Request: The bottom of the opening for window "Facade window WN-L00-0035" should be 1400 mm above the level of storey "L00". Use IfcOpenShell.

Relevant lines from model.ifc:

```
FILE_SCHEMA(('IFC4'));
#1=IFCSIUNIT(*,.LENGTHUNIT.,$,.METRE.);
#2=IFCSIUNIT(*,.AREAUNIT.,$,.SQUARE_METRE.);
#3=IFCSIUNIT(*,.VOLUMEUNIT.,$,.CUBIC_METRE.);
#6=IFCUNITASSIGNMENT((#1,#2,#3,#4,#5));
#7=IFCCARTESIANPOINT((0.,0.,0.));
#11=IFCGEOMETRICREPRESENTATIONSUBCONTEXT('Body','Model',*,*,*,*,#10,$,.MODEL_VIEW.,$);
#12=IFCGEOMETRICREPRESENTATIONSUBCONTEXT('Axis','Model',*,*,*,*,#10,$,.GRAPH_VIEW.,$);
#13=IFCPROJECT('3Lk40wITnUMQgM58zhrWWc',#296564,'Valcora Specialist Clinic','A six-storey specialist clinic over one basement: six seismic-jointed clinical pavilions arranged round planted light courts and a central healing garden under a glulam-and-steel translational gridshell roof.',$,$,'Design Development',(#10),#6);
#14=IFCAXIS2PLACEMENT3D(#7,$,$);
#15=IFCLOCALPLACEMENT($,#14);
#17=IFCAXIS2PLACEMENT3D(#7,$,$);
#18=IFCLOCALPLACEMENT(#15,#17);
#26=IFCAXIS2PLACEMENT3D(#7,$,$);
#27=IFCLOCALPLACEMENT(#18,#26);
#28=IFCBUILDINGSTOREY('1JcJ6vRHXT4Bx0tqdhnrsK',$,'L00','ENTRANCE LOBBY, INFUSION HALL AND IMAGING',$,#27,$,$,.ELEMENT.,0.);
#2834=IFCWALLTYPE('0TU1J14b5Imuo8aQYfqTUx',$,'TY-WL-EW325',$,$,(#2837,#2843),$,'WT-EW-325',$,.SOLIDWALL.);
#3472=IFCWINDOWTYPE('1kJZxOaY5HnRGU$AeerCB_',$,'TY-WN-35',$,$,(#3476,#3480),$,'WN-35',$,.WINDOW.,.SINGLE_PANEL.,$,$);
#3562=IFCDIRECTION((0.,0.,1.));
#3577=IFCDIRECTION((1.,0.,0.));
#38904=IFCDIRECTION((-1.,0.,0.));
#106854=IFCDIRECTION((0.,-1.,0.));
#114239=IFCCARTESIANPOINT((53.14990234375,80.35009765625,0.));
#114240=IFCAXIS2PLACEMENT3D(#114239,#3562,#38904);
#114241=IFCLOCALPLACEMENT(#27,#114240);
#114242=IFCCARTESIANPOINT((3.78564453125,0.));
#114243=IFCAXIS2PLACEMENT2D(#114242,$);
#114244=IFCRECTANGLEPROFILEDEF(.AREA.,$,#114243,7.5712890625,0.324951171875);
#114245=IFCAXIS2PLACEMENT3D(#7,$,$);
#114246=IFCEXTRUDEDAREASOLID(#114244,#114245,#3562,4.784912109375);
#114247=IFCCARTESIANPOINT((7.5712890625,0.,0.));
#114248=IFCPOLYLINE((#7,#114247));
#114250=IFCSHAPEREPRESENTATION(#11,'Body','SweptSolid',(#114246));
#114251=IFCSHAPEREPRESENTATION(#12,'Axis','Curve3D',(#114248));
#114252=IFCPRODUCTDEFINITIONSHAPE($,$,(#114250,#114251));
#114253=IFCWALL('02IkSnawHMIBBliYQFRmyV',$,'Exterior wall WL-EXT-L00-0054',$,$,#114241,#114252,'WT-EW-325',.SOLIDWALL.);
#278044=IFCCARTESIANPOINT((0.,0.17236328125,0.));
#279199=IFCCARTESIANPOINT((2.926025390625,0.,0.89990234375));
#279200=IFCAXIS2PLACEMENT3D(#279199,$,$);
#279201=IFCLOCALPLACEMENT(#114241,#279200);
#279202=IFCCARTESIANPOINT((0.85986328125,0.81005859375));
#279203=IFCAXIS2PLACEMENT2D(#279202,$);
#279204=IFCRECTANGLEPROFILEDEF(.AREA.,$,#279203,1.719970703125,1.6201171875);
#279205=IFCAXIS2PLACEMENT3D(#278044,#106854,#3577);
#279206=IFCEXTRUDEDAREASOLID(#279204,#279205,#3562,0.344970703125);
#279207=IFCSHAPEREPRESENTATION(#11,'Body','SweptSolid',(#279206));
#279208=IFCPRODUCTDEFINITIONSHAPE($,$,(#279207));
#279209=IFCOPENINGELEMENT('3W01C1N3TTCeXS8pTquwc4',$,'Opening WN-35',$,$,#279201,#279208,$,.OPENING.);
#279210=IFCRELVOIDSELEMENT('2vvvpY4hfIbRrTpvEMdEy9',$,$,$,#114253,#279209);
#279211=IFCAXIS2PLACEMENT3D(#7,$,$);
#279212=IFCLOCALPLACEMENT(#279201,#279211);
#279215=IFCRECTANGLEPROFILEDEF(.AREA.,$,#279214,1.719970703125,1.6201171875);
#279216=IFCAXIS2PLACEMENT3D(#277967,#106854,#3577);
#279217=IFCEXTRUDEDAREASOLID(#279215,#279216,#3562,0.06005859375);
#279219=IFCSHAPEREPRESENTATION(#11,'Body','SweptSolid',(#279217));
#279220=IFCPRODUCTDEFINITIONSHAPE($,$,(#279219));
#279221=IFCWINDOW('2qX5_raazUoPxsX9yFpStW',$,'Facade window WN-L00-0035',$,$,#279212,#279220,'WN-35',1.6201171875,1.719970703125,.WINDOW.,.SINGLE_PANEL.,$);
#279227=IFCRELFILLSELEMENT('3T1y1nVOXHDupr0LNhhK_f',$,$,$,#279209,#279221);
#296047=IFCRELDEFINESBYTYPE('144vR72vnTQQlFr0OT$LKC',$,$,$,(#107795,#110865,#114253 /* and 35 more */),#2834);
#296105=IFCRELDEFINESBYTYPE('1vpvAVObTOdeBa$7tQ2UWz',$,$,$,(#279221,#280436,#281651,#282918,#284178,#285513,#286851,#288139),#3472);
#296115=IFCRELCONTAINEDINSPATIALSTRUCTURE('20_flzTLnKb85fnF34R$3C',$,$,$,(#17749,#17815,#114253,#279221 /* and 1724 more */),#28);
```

```python
import numpy as np
import ifcopenshell
import ifcopenshell.api.geometry
import ifcopenshell.geom
import ifcopenshell.util.element
import ifcopenshell.util.placement
import ifcopenshell.util.shape
import ifcopenshell.util.unit

model = ifcopenshell.open("model.ifc")
unit_scale = ifcopenshell.util.unit.calculate_unit_scale(model)

window = model.by_guid("2qX5_raazUoPxsX9yFpStW")
opening = window.FillsVoids[0].RelatingOpeningElement
storey = ifcopenshell.util.element.get_container(window, ifc_class="IfcBuildingStorey")
level = ifcopenshell.util.placement.get_local_placement(storey.ObjectPlacement)[2, 3]

# The opening's origin need not be at the sill, so measure its lowest point.
shape = ifcopenshell.geom.create_shape(ifcopenshell.geom.settings(), opening)
bottom = ifcopenshell.util.shape.get_shape_bottom_elevation(shape, shape.geometry) / unit_scale
dz = level + 1.4 - bottom

shift = np.array([0.0, 0.0, dz])
# The window is placed relative to its opening, so it follows when the opening moves.
matrix = ifcopenshell.util.placement.get_local_placement(opening.ObjectPlacement)
matrix[:3, 3] += shift
ifcopenshell.api.geometry.edit_object_placement(
    model, product=opening, matrix=matrix, is_si=False, should_transform_children=True
)

print(f"moved by {dz * unit_scale:+.3f} m")

model.write("model-out.ifc")
```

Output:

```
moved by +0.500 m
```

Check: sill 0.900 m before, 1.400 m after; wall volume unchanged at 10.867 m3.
